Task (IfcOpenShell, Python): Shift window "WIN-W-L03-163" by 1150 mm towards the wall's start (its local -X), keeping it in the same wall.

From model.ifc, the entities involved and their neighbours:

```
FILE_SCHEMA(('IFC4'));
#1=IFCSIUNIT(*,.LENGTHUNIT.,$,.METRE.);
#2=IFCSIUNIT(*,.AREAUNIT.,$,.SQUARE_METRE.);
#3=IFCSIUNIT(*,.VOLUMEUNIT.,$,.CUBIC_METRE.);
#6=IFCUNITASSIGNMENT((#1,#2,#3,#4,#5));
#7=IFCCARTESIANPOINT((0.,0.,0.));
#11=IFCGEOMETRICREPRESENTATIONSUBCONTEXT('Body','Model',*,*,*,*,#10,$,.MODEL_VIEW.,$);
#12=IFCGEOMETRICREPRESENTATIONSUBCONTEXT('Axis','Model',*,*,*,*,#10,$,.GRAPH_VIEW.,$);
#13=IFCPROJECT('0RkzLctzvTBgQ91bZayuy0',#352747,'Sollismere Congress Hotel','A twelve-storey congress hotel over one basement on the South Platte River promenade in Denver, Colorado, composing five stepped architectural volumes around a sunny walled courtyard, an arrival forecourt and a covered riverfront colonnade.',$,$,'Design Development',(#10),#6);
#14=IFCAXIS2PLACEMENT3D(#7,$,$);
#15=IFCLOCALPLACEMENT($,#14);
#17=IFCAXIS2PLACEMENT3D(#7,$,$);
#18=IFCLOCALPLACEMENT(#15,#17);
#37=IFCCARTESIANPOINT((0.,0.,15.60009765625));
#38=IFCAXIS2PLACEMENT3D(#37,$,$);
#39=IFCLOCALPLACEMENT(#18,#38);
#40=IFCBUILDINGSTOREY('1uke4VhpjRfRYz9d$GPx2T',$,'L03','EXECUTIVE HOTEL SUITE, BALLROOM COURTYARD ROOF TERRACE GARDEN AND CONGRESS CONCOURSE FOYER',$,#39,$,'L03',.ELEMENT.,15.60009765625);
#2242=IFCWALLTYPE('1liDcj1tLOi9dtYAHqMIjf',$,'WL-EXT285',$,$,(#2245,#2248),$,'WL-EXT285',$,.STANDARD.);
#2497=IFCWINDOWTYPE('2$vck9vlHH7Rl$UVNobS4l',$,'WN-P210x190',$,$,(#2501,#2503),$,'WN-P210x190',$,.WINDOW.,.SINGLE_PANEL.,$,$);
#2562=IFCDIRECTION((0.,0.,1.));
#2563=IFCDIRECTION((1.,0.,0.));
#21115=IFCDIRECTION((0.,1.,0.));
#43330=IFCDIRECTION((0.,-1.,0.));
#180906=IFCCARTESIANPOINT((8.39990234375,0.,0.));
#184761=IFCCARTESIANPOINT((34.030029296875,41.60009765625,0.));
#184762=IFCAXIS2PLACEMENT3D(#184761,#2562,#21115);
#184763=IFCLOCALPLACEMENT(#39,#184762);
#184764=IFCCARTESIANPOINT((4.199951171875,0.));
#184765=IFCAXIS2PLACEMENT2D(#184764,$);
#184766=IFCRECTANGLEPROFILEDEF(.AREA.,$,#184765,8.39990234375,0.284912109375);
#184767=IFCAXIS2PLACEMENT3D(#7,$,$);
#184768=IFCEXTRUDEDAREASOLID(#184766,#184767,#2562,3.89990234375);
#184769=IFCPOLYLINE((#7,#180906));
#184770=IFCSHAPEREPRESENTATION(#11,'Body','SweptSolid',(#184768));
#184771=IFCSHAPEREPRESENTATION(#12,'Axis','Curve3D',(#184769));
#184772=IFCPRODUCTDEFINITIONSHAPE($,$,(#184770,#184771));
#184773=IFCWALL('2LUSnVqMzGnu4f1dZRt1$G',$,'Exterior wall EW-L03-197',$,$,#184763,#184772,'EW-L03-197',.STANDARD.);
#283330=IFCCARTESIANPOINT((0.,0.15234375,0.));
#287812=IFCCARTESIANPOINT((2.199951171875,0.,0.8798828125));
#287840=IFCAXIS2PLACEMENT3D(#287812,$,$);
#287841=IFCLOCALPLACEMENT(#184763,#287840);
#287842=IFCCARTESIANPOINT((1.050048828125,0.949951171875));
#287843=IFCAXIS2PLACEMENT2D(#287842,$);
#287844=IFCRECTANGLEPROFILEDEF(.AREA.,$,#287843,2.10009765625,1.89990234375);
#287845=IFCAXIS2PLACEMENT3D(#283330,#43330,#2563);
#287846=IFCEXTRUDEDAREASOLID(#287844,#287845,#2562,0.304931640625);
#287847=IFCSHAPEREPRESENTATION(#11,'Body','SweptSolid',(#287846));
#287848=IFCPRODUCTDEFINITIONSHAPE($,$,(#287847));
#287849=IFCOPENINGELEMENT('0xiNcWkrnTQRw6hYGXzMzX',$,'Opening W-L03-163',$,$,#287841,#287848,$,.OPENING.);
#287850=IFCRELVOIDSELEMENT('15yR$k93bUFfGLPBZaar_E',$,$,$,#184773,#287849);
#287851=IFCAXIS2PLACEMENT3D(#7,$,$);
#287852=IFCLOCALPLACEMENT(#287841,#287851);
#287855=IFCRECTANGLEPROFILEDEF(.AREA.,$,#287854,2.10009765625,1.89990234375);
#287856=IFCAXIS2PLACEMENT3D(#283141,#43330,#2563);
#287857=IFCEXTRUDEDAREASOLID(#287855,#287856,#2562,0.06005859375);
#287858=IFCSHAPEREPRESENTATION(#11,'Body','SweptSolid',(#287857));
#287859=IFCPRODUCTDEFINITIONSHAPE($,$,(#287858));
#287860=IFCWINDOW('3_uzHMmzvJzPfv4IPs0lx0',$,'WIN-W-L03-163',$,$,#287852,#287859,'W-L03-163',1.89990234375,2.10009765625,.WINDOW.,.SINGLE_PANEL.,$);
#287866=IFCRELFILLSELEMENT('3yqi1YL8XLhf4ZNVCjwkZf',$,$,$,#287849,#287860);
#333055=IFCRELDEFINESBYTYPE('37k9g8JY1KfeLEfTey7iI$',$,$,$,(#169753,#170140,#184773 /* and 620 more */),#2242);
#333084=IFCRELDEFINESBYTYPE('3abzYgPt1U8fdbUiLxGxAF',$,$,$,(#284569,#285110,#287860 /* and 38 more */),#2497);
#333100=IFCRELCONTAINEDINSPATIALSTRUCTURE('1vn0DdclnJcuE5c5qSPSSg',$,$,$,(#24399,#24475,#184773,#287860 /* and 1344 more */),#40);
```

```python
import ifcopenshell
import ifcopenshell.api.geometry
import ifcopenshell.util.placement

model = ifcopenshell.open("model.ifc")

window = model.by_id(287860)
opening = window.FillsVoids[0].RelatingOpeningElement
wall = opening.VoidsElements[0].RelatingBuildingElement

wall_matrix = ifcopenshell.util.placement.get_local_placement(wall.ObjectPlacement)
shift = wall_matrix[:3, 0] * -1.15
before = ifcopenshell.util.placement.get_local_placement(window.ObjectPlacement)[:3, 3].copy()

# The window is placed relative to its opening, so it follows when the opening moves.
matrix = ifcopenshell.util.placement.get_local_placement(opening.ObjectPlacement)
matrix[:3, 3] += shift
ifcopenshell.api.geometry.edit_object_placement(
    model, product=opening, matrix=matrix, is_si=False, should_transform_children=True
)

after = ifcopenshell.util.placement.get_local_placement(window.ObjectPlacement)[:3, 3]
print("window moved by", (after - before).round(3) + 0.0)

model.write("model_edited.ifc")
```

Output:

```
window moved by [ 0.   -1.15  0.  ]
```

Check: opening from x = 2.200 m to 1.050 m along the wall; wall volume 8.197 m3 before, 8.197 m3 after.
